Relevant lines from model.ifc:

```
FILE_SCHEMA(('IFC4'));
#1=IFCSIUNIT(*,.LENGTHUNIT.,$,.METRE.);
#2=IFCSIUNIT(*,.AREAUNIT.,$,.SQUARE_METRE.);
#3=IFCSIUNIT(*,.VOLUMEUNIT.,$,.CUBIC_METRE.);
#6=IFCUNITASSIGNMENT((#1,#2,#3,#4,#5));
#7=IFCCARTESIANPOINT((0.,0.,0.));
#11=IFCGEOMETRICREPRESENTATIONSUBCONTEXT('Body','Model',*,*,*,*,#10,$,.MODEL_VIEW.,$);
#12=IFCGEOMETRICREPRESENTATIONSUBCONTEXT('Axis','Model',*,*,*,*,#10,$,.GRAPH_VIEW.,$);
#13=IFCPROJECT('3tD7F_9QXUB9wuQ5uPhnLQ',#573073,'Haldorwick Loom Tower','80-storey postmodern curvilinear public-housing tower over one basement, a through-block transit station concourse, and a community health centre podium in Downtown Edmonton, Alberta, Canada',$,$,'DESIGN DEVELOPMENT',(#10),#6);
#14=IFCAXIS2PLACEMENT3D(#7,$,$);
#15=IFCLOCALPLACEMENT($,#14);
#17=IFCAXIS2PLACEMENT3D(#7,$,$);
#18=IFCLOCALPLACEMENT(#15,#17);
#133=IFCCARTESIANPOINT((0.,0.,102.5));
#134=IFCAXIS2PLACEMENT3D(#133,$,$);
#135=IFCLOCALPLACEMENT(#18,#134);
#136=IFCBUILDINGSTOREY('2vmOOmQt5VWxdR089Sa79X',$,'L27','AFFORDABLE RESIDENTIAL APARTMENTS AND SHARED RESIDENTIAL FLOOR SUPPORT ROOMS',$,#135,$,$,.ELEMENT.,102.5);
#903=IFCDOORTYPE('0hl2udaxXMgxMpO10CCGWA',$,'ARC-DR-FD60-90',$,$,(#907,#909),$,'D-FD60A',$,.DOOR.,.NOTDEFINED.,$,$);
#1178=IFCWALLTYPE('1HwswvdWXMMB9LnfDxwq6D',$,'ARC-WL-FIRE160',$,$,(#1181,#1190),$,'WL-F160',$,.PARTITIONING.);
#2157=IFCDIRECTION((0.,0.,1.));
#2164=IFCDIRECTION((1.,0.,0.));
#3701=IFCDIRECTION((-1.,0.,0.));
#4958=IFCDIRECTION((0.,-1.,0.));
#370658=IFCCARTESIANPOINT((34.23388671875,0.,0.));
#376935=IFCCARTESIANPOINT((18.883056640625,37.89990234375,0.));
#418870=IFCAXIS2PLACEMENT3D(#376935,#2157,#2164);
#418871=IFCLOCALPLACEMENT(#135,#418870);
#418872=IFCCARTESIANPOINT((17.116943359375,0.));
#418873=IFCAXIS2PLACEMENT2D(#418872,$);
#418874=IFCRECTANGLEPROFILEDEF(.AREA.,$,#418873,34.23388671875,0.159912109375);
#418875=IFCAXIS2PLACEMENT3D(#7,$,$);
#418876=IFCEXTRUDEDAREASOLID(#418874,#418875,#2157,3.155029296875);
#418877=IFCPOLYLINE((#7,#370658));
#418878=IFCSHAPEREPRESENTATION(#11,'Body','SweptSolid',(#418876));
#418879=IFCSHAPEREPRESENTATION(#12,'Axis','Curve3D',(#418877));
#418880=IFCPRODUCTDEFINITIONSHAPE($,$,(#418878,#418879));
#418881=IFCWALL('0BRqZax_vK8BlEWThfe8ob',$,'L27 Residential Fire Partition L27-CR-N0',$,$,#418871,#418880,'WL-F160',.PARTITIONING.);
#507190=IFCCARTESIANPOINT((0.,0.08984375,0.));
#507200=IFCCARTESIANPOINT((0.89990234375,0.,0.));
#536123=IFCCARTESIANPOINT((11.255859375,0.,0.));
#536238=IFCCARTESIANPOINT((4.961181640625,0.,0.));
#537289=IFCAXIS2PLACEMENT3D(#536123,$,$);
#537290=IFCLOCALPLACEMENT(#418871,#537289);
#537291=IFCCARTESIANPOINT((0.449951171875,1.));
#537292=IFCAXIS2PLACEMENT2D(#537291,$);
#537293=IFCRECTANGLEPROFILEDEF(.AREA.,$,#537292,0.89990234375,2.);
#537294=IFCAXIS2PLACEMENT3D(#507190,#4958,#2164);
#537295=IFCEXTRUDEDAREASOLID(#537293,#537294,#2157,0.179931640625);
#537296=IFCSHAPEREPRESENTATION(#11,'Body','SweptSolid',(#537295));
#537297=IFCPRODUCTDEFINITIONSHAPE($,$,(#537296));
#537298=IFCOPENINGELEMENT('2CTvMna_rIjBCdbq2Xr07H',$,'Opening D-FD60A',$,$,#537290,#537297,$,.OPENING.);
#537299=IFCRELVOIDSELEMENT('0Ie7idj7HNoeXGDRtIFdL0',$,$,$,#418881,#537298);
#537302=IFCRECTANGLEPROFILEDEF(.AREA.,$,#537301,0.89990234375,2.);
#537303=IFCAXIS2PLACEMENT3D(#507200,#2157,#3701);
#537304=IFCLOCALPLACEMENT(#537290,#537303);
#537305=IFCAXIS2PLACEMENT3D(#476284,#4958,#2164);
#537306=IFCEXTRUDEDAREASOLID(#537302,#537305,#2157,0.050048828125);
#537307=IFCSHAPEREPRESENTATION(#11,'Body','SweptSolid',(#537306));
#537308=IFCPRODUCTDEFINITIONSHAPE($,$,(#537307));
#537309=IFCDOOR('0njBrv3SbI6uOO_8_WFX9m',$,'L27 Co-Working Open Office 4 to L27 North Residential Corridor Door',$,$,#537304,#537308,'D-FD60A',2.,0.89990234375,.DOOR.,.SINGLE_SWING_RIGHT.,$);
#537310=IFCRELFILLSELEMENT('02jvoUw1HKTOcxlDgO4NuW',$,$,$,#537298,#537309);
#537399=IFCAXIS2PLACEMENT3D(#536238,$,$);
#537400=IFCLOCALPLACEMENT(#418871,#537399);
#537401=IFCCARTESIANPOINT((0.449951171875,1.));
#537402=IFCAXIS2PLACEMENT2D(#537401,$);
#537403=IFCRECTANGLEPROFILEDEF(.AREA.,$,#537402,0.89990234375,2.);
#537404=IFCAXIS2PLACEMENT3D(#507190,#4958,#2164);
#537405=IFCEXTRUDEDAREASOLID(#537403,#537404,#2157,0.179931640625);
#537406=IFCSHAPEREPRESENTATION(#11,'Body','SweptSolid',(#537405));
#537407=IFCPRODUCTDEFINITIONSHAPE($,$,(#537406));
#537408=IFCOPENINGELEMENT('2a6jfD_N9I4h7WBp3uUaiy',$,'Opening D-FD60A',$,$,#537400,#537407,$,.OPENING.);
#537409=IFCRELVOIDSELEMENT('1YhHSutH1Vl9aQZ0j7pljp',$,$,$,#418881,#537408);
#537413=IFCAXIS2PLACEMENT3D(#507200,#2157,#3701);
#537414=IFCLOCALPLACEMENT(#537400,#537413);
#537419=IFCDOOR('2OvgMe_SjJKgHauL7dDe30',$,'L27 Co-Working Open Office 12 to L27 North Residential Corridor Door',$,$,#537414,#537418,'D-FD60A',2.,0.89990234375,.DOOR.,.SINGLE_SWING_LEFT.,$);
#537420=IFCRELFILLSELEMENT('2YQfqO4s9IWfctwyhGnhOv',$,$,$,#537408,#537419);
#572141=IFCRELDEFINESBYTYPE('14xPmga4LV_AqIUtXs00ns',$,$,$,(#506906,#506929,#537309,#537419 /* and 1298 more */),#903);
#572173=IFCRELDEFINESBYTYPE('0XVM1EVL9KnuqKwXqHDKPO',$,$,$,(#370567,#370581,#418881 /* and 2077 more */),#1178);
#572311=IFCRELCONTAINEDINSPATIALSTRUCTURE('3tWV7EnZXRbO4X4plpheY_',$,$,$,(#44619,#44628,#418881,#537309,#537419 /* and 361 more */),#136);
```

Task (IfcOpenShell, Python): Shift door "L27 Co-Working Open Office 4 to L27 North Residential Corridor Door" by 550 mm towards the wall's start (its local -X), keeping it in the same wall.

```python
import ifcopenshell
import ifcopenshell.api.geometry
import ifcopenshell.util.placement

model = ifcopenshell.open("model.ifc")

door = model.by_guid("0njBrv3SbI6uOO_8_WFX9m")
opening = door.FillsVoids[0].RelatingOpeningElement
wall = opening.VoidsElements[0].RelatingBuildingElement

wall_matrix = ifcopenshell.util.placement.get_local_placement(wall.ObjectPlacement)
shift = wall_matrix[:3, 0] * -0.55
before = ifcopenshell.util.placement.get_local_placement(door.ObjectPlacement)[:3, 3].copy()

# The door is placed relative to its opening, so it follows when the opening moves.
matrix = ifcopenshell.util.placement.get_local_placement(opening.ObjectPlacement)
matrix[:3, 3] += shift
ifcopenshell.api.geometry.edit_object_placement(
    model, product=opening, matrix=matrix, is_si=False, should_transform_children=True
)

after = ifcopenshell.util.placement.get_local_placement(door.ObjectPlacement)[:3, 3]
print("door moved by", (after - before).round(3) + 0.0)

model.write("model_v2.ifc")
```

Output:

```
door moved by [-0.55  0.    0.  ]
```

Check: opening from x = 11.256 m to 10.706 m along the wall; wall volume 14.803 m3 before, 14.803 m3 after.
